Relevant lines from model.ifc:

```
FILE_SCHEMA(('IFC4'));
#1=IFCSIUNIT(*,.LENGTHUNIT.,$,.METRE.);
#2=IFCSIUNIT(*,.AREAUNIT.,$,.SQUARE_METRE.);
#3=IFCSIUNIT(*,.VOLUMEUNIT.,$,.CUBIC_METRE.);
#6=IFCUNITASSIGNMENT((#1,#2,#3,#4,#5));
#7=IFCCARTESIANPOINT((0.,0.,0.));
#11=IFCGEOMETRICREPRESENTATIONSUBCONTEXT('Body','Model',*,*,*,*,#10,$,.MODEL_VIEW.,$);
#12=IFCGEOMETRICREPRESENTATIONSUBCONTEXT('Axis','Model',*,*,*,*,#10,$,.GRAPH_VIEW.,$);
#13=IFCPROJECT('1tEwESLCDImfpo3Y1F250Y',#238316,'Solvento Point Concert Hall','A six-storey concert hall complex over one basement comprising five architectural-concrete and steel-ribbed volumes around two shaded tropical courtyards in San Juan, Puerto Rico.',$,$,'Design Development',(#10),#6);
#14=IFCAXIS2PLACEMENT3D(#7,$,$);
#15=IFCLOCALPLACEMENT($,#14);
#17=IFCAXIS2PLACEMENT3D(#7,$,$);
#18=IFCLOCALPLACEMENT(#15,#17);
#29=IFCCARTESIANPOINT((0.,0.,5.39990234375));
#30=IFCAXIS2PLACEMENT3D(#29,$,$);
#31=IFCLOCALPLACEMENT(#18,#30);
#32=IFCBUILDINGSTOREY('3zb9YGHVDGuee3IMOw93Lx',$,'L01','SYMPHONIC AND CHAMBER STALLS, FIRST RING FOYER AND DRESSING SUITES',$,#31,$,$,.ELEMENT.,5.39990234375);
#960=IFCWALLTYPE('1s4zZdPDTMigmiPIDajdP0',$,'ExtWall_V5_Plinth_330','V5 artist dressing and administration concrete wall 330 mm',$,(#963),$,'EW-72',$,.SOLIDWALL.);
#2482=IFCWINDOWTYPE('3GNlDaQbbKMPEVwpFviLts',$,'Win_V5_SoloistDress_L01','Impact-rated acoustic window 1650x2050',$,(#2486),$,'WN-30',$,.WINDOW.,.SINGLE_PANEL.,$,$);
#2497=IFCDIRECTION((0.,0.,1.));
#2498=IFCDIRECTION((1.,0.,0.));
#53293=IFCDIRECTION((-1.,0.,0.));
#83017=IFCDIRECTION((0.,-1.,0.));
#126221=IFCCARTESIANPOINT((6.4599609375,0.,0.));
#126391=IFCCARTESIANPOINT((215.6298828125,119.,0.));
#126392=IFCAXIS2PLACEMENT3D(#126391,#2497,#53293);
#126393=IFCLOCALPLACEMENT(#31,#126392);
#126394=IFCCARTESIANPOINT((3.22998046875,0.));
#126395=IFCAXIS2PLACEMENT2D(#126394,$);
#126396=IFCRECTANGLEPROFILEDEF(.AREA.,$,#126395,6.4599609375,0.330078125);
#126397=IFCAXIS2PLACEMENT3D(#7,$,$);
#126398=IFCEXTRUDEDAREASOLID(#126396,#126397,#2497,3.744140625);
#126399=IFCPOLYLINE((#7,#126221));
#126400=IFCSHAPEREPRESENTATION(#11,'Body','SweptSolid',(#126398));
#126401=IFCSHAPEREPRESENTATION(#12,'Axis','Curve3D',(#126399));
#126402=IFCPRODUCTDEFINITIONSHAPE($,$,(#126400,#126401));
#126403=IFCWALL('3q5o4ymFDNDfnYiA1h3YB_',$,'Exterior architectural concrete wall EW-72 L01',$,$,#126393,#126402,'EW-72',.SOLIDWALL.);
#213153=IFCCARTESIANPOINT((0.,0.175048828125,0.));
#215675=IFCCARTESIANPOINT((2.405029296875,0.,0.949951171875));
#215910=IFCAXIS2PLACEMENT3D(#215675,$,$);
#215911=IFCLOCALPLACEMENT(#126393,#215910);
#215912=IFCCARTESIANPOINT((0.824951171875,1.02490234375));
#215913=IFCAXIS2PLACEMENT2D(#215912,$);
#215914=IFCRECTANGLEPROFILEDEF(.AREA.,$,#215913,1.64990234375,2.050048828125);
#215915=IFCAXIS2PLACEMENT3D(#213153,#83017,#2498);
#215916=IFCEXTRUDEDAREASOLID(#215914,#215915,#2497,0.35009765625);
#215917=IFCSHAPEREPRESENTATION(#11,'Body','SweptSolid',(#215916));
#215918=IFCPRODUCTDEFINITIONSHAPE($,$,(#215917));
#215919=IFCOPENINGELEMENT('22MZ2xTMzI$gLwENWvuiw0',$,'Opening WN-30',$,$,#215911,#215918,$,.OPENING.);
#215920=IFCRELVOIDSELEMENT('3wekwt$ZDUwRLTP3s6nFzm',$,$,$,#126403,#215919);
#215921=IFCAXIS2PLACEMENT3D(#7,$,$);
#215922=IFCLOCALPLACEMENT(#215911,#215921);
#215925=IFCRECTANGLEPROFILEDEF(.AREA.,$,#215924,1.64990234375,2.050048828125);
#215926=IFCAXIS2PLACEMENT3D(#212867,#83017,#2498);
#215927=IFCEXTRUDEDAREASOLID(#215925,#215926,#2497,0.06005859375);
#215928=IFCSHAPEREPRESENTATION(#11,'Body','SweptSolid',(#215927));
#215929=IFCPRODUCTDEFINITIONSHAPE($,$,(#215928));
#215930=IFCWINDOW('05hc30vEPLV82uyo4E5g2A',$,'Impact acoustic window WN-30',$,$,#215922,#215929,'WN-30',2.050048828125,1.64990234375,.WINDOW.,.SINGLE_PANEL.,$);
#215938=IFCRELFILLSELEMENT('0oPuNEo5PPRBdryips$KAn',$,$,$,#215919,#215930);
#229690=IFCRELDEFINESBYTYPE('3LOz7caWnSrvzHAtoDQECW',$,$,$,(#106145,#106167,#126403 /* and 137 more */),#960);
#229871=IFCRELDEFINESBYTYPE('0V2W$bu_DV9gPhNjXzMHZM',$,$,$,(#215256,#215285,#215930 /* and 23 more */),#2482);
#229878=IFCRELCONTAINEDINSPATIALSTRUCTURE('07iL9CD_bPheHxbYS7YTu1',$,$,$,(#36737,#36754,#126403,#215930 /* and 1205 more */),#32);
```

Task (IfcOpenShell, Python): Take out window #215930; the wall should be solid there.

```python
import ifcopenshell
import ifcopenshell.api.feature
import ifcopenshell.api.root
import ifcopenshell.geom
import ifcopenshell.util.shape

model = ifcopenshell.open("model.ifc")
settings = ifcopenshell.geom.settings()


def volume(element):
    """Net volume in cubic metres, openings subtracted."""
    shape = ifcopenshell.geom.create_shape(settings, element)
    return ifcopenshell.util.shape.get_volume(shape.geometry)


window = model.by_id(215930)
opening = window.FillsVoids[0].RelatingOpeningElement
wall = opening.VoidsElements[0].RelatingBuildingElement
before = volume(wall)

ifcopenshell.api.root.remove_product(model, product=window)
ifcopenshell.api.feature.remove_feature(model, feature=opening)

after = volume(wall)

print(f"wall volume {before:.3f} -> {after:.3f} m3")

model.write("model_v2.ifc")
```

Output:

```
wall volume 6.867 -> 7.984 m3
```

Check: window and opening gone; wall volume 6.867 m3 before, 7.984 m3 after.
